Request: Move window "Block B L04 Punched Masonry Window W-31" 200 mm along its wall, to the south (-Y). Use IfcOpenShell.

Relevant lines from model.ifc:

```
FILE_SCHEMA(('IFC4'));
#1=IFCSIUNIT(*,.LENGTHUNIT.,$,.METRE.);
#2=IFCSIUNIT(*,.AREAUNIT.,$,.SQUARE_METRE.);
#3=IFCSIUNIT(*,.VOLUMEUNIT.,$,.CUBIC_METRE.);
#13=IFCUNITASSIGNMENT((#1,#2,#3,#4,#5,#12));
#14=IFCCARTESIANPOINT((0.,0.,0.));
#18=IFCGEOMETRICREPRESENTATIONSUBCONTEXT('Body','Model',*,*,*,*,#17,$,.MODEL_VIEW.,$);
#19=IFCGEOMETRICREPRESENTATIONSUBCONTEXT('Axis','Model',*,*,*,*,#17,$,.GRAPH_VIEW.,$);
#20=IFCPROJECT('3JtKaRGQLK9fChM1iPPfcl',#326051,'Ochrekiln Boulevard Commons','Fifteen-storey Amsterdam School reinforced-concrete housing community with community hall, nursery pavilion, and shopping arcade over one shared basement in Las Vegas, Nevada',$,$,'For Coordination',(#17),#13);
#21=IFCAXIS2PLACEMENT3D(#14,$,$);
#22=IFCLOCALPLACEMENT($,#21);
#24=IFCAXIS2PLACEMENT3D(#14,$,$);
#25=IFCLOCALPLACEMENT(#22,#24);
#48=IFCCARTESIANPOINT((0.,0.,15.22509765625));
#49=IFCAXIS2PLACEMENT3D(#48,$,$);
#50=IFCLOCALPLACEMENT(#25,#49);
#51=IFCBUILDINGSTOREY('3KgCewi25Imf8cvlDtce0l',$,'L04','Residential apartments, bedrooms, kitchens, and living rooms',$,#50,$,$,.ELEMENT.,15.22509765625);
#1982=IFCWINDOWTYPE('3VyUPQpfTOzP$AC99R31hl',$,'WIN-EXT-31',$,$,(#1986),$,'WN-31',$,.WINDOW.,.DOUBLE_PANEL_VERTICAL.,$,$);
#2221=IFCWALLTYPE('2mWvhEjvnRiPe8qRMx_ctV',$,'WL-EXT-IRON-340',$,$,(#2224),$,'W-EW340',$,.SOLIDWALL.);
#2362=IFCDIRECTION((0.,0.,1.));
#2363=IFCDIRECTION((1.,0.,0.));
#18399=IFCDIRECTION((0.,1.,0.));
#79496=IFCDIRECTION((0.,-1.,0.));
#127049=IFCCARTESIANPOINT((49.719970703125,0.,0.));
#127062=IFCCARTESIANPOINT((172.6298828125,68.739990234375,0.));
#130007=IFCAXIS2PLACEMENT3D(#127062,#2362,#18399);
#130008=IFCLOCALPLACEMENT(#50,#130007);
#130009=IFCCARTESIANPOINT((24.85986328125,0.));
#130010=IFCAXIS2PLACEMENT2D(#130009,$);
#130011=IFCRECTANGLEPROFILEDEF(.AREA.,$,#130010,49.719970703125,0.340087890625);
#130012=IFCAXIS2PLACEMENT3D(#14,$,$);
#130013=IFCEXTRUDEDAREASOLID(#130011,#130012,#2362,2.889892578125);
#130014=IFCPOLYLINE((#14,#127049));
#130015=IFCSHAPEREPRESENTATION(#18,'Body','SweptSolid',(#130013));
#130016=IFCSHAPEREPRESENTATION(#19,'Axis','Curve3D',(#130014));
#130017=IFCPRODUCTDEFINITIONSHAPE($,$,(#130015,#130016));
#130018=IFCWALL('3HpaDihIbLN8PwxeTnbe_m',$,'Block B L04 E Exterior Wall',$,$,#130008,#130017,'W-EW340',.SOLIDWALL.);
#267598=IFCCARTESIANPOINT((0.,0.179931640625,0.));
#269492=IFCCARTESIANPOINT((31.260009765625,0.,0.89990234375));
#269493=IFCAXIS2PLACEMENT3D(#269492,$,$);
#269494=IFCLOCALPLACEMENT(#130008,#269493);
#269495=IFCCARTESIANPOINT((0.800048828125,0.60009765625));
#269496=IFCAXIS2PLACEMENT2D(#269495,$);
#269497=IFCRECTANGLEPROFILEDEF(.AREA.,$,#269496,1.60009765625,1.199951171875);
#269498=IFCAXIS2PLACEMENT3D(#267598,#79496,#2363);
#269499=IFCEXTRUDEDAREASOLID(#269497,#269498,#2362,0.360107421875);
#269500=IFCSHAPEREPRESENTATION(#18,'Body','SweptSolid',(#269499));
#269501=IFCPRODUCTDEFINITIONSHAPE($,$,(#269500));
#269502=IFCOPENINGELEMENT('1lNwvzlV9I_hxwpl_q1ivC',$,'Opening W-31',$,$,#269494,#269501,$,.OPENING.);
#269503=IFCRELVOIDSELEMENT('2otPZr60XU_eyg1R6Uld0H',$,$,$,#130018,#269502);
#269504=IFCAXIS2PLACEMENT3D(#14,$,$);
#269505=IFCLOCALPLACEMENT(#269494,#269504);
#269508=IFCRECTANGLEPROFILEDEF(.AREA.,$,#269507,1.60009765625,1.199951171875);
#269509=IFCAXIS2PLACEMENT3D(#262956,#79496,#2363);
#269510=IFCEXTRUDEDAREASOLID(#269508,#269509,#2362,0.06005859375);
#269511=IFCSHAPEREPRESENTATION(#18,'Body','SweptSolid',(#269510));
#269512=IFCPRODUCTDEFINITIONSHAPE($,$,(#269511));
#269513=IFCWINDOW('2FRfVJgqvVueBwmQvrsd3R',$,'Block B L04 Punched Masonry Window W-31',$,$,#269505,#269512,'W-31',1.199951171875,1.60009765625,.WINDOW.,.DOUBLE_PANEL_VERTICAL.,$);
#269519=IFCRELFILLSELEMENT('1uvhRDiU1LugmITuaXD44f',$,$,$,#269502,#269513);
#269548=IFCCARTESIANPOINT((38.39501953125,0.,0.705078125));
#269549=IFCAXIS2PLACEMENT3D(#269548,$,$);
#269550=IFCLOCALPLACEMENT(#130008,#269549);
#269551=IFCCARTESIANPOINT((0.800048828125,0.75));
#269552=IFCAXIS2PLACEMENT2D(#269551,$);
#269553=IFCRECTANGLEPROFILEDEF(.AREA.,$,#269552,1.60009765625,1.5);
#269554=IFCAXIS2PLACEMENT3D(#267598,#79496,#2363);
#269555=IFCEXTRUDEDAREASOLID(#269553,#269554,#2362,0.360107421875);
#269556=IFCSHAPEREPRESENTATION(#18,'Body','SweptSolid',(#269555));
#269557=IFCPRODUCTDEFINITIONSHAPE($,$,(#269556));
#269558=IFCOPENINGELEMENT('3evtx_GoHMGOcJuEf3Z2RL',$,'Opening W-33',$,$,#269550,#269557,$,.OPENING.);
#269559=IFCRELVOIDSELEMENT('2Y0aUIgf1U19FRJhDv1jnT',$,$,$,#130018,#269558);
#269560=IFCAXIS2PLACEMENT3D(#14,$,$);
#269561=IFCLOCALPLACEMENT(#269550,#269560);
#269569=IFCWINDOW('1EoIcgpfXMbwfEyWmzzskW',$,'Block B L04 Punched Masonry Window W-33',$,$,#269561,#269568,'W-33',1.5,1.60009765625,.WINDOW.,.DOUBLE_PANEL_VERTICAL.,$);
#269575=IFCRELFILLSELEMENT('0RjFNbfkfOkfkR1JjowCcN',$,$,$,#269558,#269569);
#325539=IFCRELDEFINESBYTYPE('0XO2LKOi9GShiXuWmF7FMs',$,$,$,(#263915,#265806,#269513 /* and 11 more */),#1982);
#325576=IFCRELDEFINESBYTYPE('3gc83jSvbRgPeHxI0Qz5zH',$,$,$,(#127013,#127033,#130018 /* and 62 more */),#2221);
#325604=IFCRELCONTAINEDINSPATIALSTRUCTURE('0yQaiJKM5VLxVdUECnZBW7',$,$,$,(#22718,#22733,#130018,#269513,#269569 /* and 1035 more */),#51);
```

```python
import ifcopenshell
import ifcopenshell.api.geometry
import ifcopenshell.util.placement
import ifcopenshell.util.unit

model = ifcopenshell.open("model.ifc")
unit_scale = ifcopenshell.util.unit.calculate_unit_scale(model)

window = model.by_guid("2FRfVJgqvVueBwmQvrsd3R")
opening = window.FillsVoids[0].RelatingOpeningElement
wall = opening.VoidsElements[0].RelatingBuildingElement

wall_matrix = ifcopenshell.util.placement.get_local_placement(wall.ObjectPlacement)
shift = wall_matrix[:3, 0] * -0.2 / unit_scale
before = ifcopenshell.util.placement.get_local_placement(window.ObjectPlacement)[:3, 3].copy()

# The window is placed relative to its opening, so it follows when the opening moves.
matrix = ifcopenshell.util.placement.get_local_placement(opening.ObjectPlacement)
matrix[:3, 3] += shift
ifcopenshell.api.geometry.edit_object_placement(
    model, product=opening, matrix=matrix, is_si=False, should_transform_children=True
)

after = ifcopenshell.util.placement.get_local_placement(window.ObjectPlacement)[:3, 3]
print("window moved by", (after - before).round(3) + 0.0)

model.write("model_v2.ifc")
```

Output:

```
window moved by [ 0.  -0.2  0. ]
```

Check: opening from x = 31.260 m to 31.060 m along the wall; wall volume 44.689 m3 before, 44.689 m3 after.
